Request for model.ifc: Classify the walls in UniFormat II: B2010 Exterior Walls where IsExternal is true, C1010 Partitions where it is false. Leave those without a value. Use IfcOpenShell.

First a look at what the model holds.

```python
import ifcopenshell
import ifcopenshell.util.element

model = ifcopenshell.open("model.ifc")
print(model.schema)
print("classifications:", [c.Name for c in model.by_type("IfcClassification")])
values = [ifcopenshell.util.element.get_pset(e, "Pset_WallCommon", "IsExternal") for e in model.by_type("IfcWall")]
for value in (True, False, None):
    print("IsExternal", value, values.count(value))
```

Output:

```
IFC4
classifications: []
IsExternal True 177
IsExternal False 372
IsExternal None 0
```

```python
import ifcopenshell
import ifcopenshell.api.classification
import ifcopenshell.util.element

model = ifcopenshell.open("model.ifc")

system = ifcopenshell.api.classification.add_classification(model, classification="UniFormat II")

walls = model.by_type("IfcWall")
external = {e: ifcopenshell.util.element.get_pset(e, "Pset_WallCommon", "IsExternal") for e in walls}
for flag, code, name in ((True, "B2010", "Exterior Walls"), (False, "C1010", "Partitions")):
    products = [e for e in walls if external[e] is flag]
    ifcopenshell.api.classification.add_reference(
        model, products=products, classification=system, identification=code, name=name
    )
    print(code, len(products))

model.write("model_v2.ifc")
```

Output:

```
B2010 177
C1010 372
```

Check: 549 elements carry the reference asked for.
